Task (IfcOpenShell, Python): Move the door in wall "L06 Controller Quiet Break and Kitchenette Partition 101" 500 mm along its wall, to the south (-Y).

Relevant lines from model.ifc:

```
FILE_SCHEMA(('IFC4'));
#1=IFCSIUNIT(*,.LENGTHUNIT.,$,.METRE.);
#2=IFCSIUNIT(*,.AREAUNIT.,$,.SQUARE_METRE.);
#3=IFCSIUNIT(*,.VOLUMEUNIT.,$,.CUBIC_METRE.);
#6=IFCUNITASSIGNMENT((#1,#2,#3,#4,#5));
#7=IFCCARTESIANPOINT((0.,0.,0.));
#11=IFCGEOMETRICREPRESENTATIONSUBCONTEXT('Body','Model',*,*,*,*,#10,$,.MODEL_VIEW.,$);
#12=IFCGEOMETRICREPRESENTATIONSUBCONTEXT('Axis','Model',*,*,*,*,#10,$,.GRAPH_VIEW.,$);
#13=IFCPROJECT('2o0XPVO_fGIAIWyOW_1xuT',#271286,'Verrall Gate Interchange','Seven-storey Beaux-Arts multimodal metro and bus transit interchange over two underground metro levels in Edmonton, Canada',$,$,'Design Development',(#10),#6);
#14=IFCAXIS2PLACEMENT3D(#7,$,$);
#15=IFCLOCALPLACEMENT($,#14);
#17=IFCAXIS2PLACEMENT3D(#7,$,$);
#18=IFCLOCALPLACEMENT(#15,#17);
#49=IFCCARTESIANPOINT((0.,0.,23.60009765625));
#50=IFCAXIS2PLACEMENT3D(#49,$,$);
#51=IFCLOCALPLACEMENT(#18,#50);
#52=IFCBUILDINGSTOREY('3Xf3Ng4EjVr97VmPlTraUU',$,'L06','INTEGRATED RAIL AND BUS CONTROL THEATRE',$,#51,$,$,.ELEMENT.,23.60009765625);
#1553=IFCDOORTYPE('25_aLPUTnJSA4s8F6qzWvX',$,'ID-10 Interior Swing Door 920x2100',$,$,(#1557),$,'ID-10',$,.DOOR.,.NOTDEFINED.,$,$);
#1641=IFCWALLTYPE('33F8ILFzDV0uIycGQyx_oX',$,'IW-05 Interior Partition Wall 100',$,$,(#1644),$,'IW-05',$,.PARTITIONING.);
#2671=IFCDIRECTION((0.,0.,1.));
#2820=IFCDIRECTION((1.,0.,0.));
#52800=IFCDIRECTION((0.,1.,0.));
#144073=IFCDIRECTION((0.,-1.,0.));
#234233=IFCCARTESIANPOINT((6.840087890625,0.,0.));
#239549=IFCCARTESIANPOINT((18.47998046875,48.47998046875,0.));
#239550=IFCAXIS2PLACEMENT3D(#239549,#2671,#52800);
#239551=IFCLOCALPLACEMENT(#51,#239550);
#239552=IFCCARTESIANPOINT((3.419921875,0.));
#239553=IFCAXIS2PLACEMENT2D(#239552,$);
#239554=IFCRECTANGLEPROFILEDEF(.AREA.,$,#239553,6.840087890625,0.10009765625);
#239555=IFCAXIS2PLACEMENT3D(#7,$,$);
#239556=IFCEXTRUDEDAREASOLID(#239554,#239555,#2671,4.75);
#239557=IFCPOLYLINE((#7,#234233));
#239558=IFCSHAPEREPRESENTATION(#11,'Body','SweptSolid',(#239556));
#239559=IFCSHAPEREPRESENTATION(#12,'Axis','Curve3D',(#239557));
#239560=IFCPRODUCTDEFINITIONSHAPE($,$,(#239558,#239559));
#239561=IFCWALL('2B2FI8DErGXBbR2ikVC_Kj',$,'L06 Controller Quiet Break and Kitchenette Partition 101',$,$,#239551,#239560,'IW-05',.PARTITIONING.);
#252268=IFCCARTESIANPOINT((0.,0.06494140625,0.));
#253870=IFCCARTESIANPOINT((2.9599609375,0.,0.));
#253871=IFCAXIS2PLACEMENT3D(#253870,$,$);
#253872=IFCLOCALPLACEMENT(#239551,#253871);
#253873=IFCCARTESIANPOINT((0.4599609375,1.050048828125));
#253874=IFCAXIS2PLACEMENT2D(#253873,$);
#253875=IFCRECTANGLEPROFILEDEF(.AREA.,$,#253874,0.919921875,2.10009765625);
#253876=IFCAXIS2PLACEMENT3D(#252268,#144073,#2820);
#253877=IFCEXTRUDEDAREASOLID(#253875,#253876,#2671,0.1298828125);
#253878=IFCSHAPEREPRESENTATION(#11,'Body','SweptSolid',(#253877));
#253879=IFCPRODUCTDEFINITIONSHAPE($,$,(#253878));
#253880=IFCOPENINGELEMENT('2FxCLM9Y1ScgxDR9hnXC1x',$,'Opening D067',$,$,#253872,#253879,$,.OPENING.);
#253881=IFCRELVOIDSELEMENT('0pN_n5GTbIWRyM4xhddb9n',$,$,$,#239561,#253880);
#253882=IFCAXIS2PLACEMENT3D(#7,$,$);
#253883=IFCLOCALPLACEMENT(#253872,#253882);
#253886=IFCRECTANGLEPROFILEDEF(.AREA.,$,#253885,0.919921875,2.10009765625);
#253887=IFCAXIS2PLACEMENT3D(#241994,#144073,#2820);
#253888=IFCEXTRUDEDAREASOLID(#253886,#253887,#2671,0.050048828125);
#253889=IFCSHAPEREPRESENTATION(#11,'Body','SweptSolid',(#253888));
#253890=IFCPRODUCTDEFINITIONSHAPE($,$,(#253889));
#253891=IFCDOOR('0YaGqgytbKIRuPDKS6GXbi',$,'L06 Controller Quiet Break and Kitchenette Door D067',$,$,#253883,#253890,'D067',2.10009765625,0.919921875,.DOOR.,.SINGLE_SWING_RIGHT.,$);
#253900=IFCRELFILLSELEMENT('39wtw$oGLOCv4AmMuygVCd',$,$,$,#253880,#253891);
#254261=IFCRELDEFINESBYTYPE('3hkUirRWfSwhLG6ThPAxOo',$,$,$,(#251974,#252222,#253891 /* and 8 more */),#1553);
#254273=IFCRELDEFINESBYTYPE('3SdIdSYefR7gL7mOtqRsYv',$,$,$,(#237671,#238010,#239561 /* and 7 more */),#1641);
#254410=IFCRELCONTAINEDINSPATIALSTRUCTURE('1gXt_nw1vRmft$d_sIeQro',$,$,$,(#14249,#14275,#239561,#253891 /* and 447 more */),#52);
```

```python
import ifcopenshell
import ifcopenshell.api.geometry
import ifcopenshell.util.placement

model = ifcopenshell.open("model.ifc")

door = model.by_guid("0YaGqgytbKIRuPDKS6GXbi")
opening = door.FillsVoids[0].RelatingOpeningElement
wall = opening.VoidsElements[0].RelatingBuildingElement

wall_matrix = ifcopenshell.util.placement.get_local_placement(wall.ObjectPlacement)
shift = wall_matrix[:3, 0] * -0.5
before = ifcopenshell.util.placement.get_local_placement(door.ObjectPlacement)[:3, 3].copy()

# The door is placed relative to its opening, so it follows when the opening moves.
matrix = ifcopenshell.util.placement.get_local_placement(opening.ObjectPlacement)
matrix[:3, 3] += shift
ifcopenshell.api.geometry.edit_object_placement(
    model, product=opening, matrix=matrix, is_si=False, should_transform_children=True
)

after = ifcopenshell.util.placement.get_local_placement(door.ObjectPlacement)[:3, 3]
print("door moved by", (after - before).round(3) + 0.0)

model.write("model_edited.ifc")
```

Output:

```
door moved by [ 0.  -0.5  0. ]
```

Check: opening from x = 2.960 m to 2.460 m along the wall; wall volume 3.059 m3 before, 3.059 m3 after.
